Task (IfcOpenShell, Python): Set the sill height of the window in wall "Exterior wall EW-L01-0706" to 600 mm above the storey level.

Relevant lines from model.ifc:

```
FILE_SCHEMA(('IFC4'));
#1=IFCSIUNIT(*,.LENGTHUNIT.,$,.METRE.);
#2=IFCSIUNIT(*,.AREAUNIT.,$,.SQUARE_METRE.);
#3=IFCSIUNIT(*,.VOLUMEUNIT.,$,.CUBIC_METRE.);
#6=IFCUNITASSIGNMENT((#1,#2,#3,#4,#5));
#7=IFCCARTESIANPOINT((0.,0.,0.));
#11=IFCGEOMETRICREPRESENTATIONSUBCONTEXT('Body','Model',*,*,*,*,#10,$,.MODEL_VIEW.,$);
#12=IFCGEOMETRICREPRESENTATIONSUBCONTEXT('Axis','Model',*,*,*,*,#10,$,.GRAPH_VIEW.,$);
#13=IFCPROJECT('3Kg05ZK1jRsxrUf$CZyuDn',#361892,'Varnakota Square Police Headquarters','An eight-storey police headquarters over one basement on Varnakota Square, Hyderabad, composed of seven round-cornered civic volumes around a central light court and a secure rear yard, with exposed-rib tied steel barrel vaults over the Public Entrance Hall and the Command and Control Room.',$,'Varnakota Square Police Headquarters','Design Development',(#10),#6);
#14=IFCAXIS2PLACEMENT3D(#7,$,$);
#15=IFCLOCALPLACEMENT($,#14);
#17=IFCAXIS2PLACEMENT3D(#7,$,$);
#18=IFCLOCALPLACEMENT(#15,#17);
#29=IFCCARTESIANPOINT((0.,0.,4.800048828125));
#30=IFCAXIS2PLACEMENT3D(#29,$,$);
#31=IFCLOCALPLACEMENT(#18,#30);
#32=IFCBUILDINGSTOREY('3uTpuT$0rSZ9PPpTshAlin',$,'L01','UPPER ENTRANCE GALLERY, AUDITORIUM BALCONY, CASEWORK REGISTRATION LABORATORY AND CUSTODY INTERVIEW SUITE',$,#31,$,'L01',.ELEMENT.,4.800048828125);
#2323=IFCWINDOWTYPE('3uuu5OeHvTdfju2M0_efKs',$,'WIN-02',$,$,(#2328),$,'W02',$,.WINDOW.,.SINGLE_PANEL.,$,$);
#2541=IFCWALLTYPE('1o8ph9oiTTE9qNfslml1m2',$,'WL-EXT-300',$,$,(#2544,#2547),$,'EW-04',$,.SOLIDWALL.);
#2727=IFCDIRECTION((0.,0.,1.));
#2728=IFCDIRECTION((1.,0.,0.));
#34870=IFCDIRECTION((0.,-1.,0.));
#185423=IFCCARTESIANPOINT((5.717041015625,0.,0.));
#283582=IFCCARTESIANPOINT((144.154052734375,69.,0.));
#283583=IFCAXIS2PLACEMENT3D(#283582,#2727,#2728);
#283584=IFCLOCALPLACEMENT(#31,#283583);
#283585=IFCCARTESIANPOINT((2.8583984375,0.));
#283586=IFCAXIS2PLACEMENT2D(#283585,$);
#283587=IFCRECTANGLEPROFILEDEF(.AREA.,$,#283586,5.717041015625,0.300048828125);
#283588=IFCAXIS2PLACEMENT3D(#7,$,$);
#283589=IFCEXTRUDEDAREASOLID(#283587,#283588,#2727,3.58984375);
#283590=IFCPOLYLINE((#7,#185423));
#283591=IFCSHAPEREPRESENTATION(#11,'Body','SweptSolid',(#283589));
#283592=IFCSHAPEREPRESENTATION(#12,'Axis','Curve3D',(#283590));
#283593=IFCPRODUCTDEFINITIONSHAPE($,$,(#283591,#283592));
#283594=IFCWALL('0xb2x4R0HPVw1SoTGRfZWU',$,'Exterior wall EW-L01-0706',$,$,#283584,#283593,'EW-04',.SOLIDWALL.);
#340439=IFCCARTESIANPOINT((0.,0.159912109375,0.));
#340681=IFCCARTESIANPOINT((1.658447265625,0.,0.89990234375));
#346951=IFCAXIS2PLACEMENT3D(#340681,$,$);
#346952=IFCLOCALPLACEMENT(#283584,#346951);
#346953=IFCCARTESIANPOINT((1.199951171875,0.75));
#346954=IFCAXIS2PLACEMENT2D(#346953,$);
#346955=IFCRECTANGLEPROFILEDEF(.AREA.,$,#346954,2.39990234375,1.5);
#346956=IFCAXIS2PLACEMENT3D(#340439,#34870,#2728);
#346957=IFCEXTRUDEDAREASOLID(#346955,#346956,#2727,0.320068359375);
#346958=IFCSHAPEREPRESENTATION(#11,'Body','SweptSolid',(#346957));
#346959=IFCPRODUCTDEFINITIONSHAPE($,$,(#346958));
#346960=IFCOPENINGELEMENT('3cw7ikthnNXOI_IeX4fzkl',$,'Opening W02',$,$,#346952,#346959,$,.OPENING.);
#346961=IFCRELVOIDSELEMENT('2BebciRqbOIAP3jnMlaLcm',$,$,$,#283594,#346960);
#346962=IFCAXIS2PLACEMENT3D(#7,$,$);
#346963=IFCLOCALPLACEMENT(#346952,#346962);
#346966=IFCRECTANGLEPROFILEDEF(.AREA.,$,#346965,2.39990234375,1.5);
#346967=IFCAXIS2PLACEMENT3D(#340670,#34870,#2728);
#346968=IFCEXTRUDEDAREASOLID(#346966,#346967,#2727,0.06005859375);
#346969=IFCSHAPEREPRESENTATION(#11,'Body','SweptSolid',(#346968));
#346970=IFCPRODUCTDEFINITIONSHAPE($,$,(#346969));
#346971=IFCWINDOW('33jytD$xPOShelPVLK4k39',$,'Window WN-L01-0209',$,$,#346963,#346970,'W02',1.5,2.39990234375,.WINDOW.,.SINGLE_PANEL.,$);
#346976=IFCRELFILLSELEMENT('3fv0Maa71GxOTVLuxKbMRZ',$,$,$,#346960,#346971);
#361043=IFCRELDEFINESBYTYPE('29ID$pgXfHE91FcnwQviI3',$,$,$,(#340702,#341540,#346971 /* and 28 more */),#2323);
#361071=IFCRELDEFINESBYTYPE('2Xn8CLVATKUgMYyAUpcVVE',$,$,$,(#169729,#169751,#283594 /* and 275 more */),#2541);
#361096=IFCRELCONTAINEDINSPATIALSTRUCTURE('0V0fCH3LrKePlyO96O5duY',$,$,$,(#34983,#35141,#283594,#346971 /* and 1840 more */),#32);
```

```python
import numpy as np
import ifcopenshell
import ifcopenshell.api.geometry
import ifcopenshell.geom
import ifcopenshell.util.element
import ifcopenshell.util.placement
import ifcopenshell.util.shape
import ifcopenshell.util.unit

model = ifcopenshell.open("model.ifc")
unit_scale = ifcopenshell.util.unit.calculate_unit_scale(model)

window = model.by_id(346971)
opening = window.FillsVoids[0].RelatingOpeningElement
storey = ifcopenshell.util.element.get_container(window, ifc_class="IfcBuildingStorey")
level = ifcopenshell.util.placement.get_local_placement(storey.ObjectPlacement)[2, 3]

# The opening's origin need not be at the sill, so measure its lowest point.
shape = ifcopenshell.geom.create_shape(ifcopenshell.geom.settings(), opening)
bottom = ifcopenshell.util.shape.get_shape_bottom_elevation(shape, shape.geometry) / unit_scale
dz = level + 0.6 - bottom

shift = np.array([0.0, 0.0, dz])
# The window is placed relative to its opening, so it follows when the opening moves.
matrix = ifcopenshell.util.placement.get_local_placement(opening.ObjectPlacement)
matrix[:3, 3] += shift
ifcopenshell.api.geometry.edit_object_placement(
    model, product=opening, matrix=matrix, is_si=False, should_transform_children=True
)

print(f"moved by {dz * unit_scale:+.3f} m")

model.write("model_v2.ifc")
```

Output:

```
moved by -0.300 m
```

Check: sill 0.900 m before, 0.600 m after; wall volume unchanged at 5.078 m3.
